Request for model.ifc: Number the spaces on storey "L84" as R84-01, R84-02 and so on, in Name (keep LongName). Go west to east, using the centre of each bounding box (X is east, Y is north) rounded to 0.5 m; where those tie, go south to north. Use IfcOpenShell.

First a look at what the model holds.

```python
import ifcopenshell
import ifcopenshell.util.element
import ifcopenshell.util.placement

model = ifcopenshell.open("model.ifc")
print(model.schema)
storey = next(s for s in model.by_type("IfcBuildingStorey") if s.Name == "L84")
spaces = [e for e in ifcopenshell.util.element.get_decomposition(storey) if e.is_a("IfcSpace")]
for e in sorted(spaces, key=lambda e: e.id()):
    origin = ifcopenshell.util.placement.get_local_placement(e.ObjectPlacement)[:3, 3]
    print(e.id(), e.Name, e.LongName, origin.round(2) + 0.0, sep=" | ")
```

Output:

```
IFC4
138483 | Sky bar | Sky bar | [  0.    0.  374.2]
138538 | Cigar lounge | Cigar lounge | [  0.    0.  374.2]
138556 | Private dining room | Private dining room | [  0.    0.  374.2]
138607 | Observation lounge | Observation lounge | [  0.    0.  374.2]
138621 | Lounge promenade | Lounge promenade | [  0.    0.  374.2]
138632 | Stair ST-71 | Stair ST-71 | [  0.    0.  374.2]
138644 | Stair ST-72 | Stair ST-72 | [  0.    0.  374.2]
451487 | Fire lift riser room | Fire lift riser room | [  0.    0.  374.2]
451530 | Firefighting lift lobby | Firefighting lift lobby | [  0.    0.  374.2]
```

```python
import ifcopenshell
import ifcopenshell.geom
import ifcopenshell.util.element
import ifcopenshell.util.shape

model = ifcopenshell.open("model.ifc")
settings = ifcopenshell.geom.settings()
settings.set("use-world-coords", True)


def centre(element):
    shape = ifcopenshell.geom.create_shape(settings, element)
    return ifcopenshell.util.shape.get_bbox_centroid(shape.geometry)


storey = next(s for s in model.by_type("IfcBuildingStorey") if s.Name == "L84")
spaces = [e for e in ifcopenshell.util.element.get_decomposition(storey) if e.is_a("IfcSpace")]

# Insertion points can sit at a corner or the storey origin, so sort by the geometry (in metres).
centres = {e: centre(e) for e in spaces}
spaces.sort(key=lambda e: (round(centres[e][0] / 0.5), centres[e][1]))

for i, e in enumerate(spaces, start=1):
    number = f"R84-{i:02d}"
    e.Name = number
    print(e.id(), number)

model.write("model_rev.ifc")
```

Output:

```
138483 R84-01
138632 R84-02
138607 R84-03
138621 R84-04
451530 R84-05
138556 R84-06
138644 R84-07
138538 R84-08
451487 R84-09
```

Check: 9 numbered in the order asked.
